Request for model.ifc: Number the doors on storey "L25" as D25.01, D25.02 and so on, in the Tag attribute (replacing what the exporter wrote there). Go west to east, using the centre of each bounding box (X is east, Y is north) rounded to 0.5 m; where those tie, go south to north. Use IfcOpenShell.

First a look at what the model holds.

```python
import ifcopenshell
import ifcopenshell.util.element
import ifcopenshell.util.placement

model = ifcopenshell.open("model.ifc")
print(model.schema)
storey = next(s for s in model.by_type("IfcBuildingStorey") if s.Name == "L25")
doors = [e for e in ifcopenshell.util.element.get_decomposition(storey) if e.is_a("IfcDoor")]
for e in sorted(doors, key=lambda e: e.id()):
    origin = ifcopenshell.util.placement.get_local_placement(e.ObjectPlacement)[:3, 3]
    print(e.id(), e.Tag, e.Name, origin.round(2) + 0.0, sep=" | ")
```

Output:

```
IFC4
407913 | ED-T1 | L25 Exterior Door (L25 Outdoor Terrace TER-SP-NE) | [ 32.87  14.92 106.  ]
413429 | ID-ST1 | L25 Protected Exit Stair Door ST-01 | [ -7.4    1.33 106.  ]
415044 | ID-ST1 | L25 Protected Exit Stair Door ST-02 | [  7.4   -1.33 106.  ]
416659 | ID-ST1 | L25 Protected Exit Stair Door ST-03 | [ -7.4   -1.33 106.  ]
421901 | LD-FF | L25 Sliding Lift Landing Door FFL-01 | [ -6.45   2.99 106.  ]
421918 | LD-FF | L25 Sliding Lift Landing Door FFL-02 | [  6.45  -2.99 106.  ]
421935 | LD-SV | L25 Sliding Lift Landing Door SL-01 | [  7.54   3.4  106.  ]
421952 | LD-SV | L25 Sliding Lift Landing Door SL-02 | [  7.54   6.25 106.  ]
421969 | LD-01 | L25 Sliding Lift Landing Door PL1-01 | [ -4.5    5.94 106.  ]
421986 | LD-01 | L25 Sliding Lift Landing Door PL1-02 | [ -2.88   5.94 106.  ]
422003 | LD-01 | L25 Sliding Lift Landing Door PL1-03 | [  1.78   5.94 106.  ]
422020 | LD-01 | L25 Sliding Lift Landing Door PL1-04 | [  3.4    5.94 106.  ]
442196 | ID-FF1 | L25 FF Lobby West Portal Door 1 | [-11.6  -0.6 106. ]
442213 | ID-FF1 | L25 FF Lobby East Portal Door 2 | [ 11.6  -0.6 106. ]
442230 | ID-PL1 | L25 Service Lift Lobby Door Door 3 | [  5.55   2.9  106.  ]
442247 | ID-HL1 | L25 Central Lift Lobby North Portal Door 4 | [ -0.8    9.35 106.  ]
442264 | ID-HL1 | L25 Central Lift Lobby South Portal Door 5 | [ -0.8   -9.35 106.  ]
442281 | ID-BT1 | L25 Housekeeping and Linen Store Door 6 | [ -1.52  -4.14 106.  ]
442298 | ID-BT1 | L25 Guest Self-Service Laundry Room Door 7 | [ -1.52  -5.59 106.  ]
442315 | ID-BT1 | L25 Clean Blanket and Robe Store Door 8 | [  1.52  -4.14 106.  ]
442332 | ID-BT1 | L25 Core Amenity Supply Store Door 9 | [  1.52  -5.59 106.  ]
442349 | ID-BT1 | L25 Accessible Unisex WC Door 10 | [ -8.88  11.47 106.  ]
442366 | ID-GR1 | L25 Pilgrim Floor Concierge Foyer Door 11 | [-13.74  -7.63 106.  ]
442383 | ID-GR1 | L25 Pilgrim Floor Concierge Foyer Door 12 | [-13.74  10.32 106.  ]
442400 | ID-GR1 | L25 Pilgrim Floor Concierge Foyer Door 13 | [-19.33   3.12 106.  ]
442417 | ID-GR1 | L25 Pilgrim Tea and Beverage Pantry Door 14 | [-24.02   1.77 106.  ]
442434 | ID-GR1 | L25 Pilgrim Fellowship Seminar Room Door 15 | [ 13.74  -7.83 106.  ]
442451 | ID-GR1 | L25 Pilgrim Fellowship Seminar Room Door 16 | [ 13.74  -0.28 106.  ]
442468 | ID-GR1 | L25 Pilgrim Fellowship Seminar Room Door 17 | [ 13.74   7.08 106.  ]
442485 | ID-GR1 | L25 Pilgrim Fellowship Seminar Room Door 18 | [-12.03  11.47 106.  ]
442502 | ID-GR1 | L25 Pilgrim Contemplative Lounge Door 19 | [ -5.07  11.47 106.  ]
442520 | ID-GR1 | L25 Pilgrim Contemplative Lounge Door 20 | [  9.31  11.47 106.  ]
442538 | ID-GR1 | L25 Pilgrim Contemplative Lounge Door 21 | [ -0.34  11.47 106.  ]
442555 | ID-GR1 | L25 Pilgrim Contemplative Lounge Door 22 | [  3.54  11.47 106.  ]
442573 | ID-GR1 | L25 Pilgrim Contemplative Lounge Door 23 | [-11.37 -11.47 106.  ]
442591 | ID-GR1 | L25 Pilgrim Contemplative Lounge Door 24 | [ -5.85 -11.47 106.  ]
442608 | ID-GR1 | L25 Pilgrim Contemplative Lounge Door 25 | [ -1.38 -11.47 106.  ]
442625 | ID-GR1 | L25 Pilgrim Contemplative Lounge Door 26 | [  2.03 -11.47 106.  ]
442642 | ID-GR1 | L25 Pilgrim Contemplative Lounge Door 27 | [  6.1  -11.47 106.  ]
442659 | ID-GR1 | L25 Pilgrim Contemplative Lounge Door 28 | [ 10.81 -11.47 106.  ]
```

```python
import ifcopenshell
import ifcopenshell.geom
import ifcopenshell.util.element
import ifcopenshell.util.shape

model = ifcopenshell.open("model.ifc")
settings = ifcopenshell.geom.settings()
settings.set("use-world-coords", True)


def centre(element):
    shape = ifcopenshell.geom.create_shape(settings, element)
    return ifcopenshell.util.shape.get_bbox_centroid(shape.geometry)


storey = next(s for s in model.by_type("IfcBuildingStorey") if s.Name == "L25")
doors = [e for e in ifcopenshell.util.element.get_decomposition(storey) if e.is_a("IfcDoor")]

# Insertion points can sit at a corner or the storey origin, so sort by the geometry (in metres).
centres = {e: centre(e) for e in doors}
doors.sort(key=lambda e: (round(centres[e][0] / 0.5), centres[e][1]))

for i, e in enumerate(doors, start=1):
    number = f"D25.{i:02d}"
    e.Tag = number
    print(e.id(), number)

model.write("model_rev.ifc")
```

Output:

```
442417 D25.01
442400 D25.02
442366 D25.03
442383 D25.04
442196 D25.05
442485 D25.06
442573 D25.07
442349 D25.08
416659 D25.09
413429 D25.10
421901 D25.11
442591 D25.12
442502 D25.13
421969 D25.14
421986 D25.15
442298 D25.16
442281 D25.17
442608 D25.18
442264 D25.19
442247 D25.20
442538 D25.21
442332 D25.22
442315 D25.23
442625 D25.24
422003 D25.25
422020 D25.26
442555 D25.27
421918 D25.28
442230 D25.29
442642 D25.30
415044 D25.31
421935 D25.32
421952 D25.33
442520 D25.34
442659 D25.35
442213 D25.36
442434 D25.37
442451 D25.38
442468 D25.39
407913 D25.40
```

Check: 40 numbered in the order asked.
